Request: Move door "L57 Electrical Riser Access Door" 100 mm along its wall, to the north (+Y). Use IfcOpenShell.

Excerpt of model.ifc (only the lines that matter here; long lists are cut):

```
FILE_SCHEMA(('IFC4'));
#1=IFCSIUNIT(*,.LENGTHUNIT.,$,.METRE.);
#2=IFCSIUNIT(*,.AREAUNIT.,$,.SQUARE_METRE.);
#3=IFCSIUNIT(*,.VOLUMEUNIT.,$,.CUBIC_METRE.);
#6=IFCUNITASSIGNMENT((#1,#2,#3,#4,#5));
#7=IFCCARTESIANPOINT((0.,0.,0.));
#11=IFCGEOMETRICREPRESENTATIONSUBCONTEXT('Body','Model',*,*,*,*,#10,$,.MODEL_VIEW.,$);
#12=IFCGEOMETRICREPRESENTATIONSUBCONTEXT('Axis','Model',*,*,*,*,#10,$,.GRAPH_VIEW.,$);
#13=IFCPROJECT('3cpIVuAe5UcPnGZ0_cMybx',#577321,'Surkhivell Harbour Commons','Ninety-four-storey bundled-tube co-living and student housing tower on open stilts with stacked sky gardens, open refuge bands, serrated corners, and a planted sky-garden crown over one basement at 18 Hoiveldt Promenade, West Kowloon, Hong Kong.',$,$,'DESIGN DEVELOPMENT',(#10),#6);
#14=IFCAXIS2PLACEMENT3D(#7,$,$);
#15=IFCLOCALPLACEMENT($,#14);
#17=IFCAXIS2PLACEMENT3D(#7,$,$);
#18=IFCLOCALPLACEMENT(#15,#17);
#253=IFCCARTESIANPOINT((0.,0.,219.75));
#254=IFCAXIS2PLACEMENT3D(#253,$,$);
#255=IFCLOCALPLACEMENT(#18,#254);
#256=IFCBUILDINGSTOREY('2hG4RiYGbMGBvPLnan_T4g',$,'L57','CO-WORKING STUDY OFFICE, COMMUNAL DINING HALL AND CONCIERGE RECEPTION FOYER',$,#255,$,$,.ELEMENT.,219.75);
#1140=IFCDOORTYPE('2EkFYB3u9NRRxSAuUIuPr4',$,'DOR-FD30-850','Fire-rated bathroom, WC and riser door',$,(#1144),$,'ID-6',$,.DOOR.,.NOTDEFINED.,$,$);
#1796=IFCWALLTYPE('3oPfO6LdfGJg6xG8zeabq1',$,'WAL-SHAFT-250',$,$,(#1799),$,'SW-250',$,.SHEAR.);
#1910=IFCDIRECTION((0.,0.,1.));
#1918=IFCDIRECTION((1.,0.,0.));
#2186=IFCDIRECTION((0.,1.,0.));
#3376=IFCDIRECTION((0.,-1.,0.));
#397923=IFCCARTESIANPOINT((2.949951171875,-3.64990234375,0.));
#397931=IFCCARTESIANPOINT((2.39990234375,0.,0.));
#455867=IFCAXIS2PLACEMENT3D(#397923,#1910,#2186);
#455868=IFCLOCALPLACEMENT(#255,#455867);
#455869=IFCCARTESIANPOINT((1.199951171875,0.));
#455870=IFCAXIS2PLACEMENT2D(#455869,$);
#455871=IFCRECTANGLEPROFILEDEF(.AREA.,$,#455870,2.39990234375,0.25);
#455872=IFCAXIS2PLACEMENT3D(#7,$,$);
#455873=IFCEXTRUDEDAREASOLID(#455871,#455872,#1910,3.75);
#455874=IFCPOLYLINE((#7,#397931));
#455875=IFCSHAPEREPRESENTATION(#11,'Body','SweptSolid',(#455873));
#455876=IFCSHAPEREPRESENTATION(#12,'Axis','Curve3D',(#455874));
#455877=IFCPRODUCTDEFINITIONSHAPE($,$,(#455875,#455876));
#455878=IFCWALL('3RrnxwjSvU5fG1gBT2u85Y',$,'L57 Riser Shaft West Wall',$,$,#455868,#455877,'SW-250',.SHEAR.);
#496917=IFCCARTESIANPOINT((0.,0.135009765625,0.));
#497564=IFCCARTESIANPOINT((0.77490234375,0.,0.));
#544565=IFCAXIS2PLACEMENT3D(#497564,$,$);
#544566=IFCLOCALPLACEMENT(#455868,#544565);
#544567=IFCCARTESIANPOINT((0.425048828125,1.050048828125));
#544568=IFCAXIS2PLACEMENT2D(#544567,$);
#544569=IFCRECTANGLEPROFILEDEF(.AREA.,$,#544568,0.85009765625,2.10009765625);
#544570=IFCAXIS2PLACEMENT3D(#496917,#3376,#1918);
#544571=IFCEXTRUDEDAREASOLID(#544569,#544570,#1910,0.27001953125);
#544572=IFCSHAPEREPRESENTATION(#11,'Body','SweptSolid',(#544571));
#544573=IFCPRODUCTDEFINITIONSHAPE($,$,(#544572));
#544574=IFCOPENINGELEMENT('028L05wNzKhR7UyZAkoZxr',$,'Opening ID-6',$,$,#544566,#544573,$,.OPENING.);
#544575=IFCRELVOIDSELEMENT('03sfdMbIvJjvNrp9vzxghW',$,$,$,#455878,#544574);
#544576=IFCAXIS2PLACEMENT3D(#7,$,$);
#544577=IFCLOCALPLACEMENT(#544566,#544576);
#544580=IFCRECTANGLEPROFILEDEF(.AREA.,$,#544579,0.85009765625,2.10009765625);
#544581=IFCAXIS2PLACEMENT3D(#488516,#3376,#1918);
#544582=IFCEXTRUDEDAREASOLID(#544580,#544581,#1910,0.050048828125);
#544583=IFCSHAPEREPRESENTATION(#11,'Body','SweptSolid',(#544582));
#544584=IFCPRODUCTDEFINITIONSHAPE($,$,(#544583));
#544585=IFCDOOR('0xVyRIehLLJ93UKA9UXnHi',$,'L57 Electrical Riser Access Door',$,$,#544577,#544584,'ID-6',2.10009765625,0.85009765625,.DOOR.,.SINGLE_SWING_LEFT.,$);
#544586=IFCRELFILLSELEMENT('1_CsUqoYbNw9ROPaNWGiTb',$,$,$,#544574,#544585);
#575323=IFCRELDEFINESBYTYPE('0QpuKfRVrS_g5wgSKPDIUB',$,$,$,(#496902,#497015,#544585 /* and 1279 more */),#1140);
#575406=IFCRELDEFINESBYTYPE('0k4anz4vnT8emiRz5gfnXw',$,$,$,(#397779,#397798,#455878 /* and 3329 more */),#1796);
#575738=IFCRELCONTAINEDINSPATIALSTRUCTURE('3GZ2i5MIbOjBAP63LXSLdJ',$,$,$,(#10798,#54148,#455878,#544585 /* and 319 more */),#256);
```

```python
import ifcopenshell
import ifcopenshell.api.geometry
import ifcopenshell.util.placement
import ifcopenshell.util.unit

model = ifcopenshell.open("model.ifc")
unit_scale = ifcopenshell.util.unit.calculate_unit_scale(model)

door = model.by_guid("0xVyRIehLLJ93UKA9UXnHi")
opening = door.FillsVoids[0].RelatingOpeningElement
wall = opening.VoidsElements[0].RelatingBuildingElement

wall_matrix = ifcopenshell.util.placement.get_local_placement(wall.ObjectPlacement)
shift = wall_matrix[:3, 0] * 0.1 / unit_scale
before = ifcopenshell.util.placement.get_local_placement(door.ObjectPlacement)[:3, 3].copy()

# The door is placed relative to its opening, so it follows when the opening moves.
matrix = ifcopenshell.util.placement.get_local_placement(opening.ObjectPlacement)
matrix[:3, 3] += shift
ifcopenshell.api.geometry.edit_object_placement(
    model, product=opening, matrix=matrix, is_si=False, should_transform_children=True
)

after = ifcopenshell.util.placement.get_local_placement(door.ObjectPlacement)[:3, 3]
print("door moved by", (after - before).round(3) + 0.0)

model.write("model_edited.ifc")
```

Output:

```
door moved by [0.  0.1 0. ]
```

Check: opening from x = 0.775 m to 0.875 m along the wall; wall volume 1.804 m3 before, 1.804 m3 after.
